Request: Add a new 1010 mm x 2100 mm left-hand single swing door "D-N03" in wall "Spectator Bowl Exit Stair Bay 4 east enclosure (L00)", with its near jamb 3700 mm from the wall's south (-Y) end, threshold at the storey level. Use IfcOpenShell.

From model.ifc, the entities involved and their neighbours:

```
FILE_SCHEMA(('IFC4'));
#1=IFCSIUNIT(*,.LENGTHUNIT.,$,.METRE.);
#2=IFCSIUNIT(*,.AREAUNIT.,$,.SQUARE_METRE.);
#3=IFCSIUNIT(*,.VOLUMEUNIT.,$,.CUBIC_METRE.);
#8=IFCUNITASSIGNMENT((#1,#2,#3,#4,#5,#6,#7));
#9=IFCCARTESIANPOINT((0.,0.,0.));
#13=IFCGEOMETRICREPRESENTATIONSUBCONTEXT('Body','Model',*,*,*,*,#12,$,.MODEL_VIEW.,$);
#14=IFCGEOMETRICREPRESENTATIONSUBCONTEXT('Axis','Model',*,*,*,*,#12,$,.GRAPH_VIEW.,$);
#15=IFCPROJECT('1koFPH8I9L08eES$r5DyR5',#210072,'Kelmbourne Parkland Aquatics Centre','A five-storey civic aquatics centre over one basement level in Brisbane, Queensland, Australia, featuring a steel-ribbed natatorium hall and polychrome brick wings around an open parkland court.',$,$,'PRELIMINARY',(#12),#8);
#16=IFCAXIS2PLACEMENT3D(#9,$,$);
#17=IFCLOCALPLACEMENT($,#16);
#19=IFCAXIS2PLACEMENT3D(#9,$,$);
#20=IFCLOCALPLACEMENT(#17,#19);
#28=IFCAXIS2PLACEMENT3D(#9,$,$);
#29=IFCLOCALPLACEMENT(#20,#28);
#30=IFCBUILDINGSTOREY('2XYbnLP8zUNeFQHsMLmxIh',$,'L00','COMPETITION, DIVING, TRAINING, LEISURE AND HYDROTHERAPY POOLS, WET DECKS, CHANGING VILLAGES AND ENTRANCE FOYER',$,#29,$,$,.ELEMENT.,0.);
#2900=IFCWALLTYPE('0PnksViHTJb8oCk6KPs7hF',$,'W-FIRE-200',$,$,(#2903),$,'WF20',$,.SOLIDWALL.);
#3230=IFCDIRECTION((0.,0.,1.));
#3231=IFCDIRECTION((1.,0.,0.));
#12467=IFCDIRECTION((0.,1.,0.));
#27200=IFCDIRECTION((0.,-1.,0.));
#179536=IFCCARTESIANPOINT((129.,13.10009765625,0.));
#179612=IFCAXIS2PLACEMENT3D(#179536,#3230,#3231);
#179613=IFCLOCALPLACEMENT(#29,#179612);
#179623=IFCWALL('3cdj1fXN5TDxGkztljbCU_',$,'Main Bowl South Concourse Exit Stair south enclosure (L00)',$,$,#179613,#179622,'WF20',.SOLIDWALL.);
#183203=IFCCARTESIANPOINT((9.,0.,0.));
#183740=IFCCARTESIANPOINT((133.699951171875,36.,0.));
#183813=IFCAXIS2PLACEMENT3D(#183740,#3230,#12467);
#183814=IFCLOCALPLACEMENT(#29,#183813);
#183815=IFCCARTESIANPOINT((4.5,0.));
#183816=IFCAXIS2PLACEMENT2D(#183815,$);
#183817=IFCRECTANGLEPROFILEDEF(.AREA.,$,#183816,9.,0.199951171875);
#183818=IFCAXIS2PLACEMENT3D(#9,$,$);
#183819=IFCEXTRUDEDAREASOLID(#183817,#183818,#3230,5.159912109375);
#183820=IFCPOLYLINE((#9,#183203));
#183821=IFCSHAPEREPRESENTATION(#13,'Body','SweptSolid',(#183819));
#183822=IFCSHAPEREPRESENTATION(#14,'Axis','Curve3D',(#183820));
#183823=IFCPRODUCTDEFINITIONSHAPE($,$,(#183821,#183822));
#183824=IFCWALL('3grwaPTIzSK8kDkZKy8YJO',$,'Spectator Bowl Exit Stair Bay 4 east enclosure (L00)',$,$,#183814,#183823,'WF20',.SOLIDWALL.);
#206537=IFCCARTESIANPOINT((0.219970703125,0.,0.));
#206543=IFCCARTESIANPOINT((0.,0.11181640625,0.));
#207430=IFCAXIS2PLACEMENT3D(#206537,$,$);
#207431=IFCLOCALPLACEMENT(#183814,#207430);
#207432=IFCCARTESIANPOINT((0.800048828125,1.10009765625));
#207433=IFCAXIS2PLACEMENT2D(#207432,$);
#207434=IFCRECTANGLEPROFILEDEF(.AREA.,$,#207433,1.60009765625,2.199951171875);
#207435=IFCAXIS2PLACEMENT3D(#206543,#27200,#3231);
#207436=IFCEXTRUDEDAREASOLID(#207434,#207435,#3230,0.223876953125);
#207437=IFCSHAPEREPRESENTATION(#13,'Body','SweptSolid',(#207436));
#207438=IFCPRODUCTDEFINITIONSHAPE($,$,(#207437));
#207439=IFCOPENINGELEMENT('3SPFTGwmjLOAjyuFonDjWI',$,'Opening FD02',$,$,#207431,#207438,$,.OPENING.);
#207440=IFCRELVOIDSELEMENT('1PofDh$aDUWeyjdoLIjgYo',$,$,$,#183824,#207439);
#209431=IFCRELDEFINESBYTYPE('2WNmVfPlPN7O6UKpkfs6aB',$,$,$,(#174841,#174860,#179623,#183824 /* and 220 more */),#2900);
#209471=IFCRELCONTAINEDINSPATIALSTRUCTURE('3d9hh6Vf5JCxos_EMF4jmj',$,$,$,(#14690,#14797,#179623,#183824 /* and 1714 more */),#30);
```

```python
import numpy as np
import ifcopenshell
import ifcopenshell.api.feature
import ifcopenshell.api.geometry
import ifcopenshell.api.root
import ifcopenshell.api.spatial
import ifcopenshell.geom
import ifcopenshell.util.element
import ifcopenshell.util.placement
import ifcopenshell.util.representation
import ifcopenshell.util.shape
import ifcopenshell.util.unit

model = ifcopenshell.open("model.ifc")
unit_scale = ifcopenshell.util.unit.calculate_unit_scale(model)
settings = ifcopenshell.geom.settings()


def volume(element):
    """Net volume in cubic metres, openings subtracted."""
    shape = ifcopenshell.geom.create_shape(settings, element)
    return ifcopenshell.util.shape.get_volume(shape.geometry)


wall = model.by_id(183824)
storey = ifcopenshell.util.element.get_container(wall, ifc_class="IfcBuildingStorey")
context = ifcopenshell.util.representation.get_context(model, "Model", "Body", "MODEL_VIEW")
before = volume(wall)

width, height, from_end, sill = 1.01, 2.1, 3.7, 0.0  # metres

# The wall runs along its own X axis, and the end named is its -X end.
wall_shape = ifcopenshell.geom.create_shape(settings, wall)
x, y, z = ifcopenshell.util.shape.get_vertices(wall_shape.geometry).T
start = x.min() + from_end
face, thickness = float(y.min()), float(y.max() - y.min())
wall_matrix = ifcopenshell.util.placement.get_local_placement(wall.ObjectPlacement)
level = ifcopenshell.util.placement.get_local_placement(storey.ObjectPlacement)[2, 3]


def in_wall(x, y):
    """Placement at x, y metres in the wall's axes, at sill height."""
    matrix = wall_matrix.copy()
    matrix[:, 3] = wall_matrix @ np.array([x / unit_scale, y / unit_scale, 0.0, 1.0])
    matrix[2, 3] = level + sill / unit_scale
    return matrix


# Opening: a box that overshoots both wall faces by 50 mm.
opening = ifcopenshell.api.root.create_entity(model, ifc_class="IfcOpeningElement", predefined_type="OPENING")
box = ifcopenshell.api.geometry.add_wall_representation(
    model, context=context, length=width, height=height, thickness=thickness + 0.1
)
ifcopenshell.api.geometry.assign_representation(model, product=opening, representation=box)
ifcopenshell.api.geometry.edit_object_placement(model, product=opening, matrix=in_wall(start, face - 0.05), is_si=False)
ifcopenshell.api.feature.add_feature(model, feature=opening, element=wall)

door = ifcopenshell.api.root.create_entity(model, ifc_class="IfcDoor", name="D-N03", predefined_type="DOOR")
door.OverallWidth, door.OverallHeight = width / unit_scale, height / unit_scale
door.OperationType = "SINGLE_SWING_LEFT"
body = ifcopenshell.api.geometry.add_door_representation(
    model,
    context=context,
    overall_width=door.OverallWidth,
    overall_height=door.OverallHeight,
    operation_type="SINGLE_SWING_LEFT",
    lining_properties={"LiningDepth": thickness / unit_scale, "ThresholdDepth": thickness / unit_scale},
)
ifcopenshell.api.geometry.assign_representation(model, product=door, representation=body)
ifcopenshell.api.spatial.assign_container(model, products=[door], relating_structure=storey)
ifcopenshell.api.feature.add_filling(model, opening=opening, element=door)

# The lining spans the wall, so the door starts at the wall face.
ifcopenshell.api.geometry.edit_object_placement(model, product=door, matrix=in_wall(start, face), is_si=False)

after = volume(wall)

print(f"wall volume {before:.3f} -> {after:.3f} m3")

model.write("model_v2.ifc")
```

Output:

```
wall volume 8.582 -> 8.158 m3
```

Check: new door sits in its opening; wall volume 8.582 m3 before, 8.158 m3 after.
